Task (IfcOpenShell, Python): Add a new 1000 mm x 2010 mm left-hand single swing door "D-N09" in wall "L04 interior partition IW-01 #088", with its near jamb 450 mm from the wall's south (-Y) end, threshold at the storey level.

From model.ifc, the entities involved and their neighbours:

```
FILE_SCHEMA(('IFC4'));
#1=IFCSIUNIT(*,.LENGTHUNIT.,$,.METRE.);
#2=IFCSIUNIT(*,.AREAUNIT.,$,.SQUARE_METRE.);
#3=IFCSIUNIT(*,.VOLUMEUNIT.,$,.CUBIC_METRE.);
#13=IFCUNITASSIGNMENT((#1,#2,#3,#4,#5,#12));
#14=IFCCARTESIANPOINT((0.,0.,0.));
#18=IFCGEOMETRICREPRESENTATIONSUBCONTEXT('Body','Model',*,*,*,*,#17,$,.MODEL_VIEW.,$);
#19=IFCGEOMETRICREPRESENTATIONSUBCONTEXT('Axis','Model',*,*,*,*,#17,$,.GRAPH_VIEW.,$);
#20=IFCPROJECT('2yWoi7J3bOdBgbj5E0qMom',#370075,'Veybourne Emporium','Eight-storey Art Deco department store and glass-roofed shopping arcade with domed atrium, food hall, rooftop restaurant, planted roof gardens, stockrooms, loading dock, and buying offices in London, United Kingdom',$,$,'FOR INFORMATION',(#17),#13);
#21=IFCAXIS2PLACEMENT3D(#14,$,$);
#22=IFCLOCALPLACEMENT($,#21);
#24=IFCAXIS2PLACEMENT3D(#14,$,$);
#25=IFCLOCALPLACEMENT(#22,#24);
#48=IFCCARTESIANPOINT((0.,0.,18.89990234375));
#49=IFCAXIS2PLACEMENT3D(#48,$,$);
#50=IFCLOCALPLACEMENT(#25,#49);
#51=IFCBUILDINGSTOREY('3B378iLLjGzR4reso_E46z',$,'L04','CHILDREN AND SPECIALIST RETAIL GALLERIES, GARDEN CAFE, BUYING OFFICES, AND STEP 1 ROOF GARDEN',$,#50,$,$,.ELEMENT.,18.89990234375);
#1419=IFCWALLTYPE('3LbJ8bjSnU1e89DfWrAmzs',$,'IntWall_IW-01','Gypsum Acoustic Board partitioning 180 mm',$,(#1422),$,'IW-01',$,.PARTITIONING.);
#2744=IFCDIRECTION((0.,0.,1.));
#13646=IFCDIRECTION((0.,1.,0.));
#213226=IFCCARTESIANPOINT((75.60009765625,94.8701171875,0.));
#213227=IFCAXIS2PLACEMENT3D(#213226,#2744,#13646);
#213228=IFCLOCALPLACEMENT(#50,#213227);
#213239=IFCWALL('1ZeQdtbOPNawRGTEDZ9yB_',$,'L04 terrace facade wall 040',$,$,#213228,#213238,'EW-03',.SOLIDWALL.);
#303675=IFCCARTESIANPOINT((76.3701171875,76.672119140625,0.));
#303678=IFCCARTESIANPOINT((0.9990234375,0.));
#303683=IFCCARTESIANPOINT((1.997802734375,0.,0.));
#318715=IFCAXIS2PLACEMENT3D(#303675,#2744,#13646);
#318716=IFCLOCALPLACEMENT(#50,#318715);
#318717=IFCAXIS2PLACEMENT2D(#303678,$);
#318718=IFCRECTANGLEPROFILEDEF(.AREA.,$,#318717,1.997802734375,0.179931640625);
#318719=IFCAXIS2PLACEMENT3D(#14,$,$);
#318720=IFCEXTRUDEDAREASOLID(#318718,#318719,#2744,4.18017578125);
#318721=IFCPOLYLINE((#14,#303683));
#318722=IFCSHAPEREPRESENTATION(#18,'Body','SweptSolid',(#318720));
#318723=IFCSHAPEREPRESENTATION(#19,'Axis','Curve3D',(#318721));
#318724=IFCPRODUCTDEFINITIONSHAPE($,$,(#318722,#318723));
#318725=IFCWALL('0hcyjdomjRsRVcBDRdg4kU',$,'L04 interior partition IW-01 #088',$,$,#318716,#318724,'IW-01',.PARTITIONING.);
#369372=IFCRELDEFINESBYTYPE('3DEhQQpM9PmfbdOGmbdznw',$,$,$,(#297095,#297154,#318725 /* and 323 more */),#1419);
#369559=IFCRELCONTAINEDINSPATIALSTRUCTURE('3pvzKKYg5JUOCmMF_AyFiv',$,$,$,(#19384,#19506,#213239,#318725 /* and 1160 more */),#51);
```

```python
import numpy as np
import ifcopenshell
import ifcopenshell.api.feature
import ifcopenshell.api.geometry
import ifcopenshell.api.root
import ifcopenshell.api.spatial
import ifcopenshell.geom
import ifcopenshell.util.element
import ifcopenshell.util.placement
import ifcopenshell.util.representation
import ifcopenshell.util.shape
import ifcopenshell.util.unit

model = ifcopenshell.open("model.ifc")
unit_scale = ifcopenshell.util.unit.calculate_unit_scale(model)
settings = ifcopenshell.geom.settings()


def volume(element):
    """Net volume in cubic metres, openings subtracted."""
    shape = ifcopenshell.geom.create_shape(settings, element)
    return ifcopenshell.util.shape.get_volume(shape.geometry)


wall = model.by_guid("0hcyjdomjRsRVcBDRdg4kU")
storey = ifcopenshell.util.element.get_container(wall, ifc_class="IfcBuildingStorey")
context = ifcopenshell.util.representation.get_context(model, "Model", "Body", "MODEL_VIEW")
before = volume(wall)

width, height, from_end, sill = 1, 2.01, 0.45, 0.0  # metres

# The wall runs along its own X axis, and the end named is its -X end.
wall_shape = ifcopenshell.geom.create_shape(settings, wall)
x, y, z = ifcopenshell.util.shape.get_vertices(wall_shape.geometry).T
start = x.min() + from_end
face, thickness = float(y.min()), float(y.max() - y.min())
wall_matrix = ifcopenshell.util.placement.get_local_placement(wall.ObjectPlacement)
level = ifcopenshell.util.placement.get_local_placement(storey.ObjectPlacement)[2, 3]


def in_wall(x, y):
    """Placement at x, y metres in the wall's axes, at sill height."""
    matrix = wall_matrix.copy()
    matrix[:, 3] = wall_matrix @ np.array([x / unit_scale, y / unit_scale, 0.0, 1.0])
    matrix[2, 3] = level + sill / unit_scale
    return matrix


# Opening: a box that overshoots both wall faces by 50 mm.
opening = ifcopenshell.api.root.create_entity(model, ifc_class="IfcOpeningElement", predefined_type="OPENING")
box = ifcopenshell.api.geometry.add_wall_representation(
    model, context=context, length=width, height=height, thickness=thickness + 0.1
)
ifcopenshell.api.geometry.assign_representation(model, product=opening, representation=box)
ifcopenshell.api.geometry.edit_object_placement(model, product=opening, matrix=in_wall(start, face - 0.05), is_si=False)
ifcopenshell.api.feature.add_feature(model, feature=opening, element=wall)

door = ifcopenshell.api.root.create_entity(model, ifc_class="IfcDoor", name="D-N09", predefined_type="DOOR")
door.OverallWidth, door.OverallHeight = width / unit_scale, height / unit_scale
door.OperationType = "SINGLE_SWING_LEFT"
body = ifcopenshell.api.geometry.add_door_representation(
    model,
    context=context,
    overall_width=door.OverallWidth,
    overall_height=door.OverallHeight,
    operation_type="SINGLE_SWING_LEFT",
    lining_properties={"LiningDepth": thickness / unit_scale, "ThresholdDepth": thickness / unit_scale},
)
ifcopenshell.api.geometry.assign_representation(model, product=door, representation=body)
ifcopenshell.api.spatial.assign_container(model, products=[door], relating_structure=storey)
ifcopenshell.api.feature.add_filling(model, opening=opening, element=door)

# The lining spans the wall, so the door starts at the wall face.
ifcopenshell.api.geometry.edit_object_placement(model, product=door, matrix=in_wall(start, face), is_si=False)

after = volume(wall)

print(f"wall volume {before:.3f} -> {after:.3f} m3")

model.write("model_rev.ifc")
```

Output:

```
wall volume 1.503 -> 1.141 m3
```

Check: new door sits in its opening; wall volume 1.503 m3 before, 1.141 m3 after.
